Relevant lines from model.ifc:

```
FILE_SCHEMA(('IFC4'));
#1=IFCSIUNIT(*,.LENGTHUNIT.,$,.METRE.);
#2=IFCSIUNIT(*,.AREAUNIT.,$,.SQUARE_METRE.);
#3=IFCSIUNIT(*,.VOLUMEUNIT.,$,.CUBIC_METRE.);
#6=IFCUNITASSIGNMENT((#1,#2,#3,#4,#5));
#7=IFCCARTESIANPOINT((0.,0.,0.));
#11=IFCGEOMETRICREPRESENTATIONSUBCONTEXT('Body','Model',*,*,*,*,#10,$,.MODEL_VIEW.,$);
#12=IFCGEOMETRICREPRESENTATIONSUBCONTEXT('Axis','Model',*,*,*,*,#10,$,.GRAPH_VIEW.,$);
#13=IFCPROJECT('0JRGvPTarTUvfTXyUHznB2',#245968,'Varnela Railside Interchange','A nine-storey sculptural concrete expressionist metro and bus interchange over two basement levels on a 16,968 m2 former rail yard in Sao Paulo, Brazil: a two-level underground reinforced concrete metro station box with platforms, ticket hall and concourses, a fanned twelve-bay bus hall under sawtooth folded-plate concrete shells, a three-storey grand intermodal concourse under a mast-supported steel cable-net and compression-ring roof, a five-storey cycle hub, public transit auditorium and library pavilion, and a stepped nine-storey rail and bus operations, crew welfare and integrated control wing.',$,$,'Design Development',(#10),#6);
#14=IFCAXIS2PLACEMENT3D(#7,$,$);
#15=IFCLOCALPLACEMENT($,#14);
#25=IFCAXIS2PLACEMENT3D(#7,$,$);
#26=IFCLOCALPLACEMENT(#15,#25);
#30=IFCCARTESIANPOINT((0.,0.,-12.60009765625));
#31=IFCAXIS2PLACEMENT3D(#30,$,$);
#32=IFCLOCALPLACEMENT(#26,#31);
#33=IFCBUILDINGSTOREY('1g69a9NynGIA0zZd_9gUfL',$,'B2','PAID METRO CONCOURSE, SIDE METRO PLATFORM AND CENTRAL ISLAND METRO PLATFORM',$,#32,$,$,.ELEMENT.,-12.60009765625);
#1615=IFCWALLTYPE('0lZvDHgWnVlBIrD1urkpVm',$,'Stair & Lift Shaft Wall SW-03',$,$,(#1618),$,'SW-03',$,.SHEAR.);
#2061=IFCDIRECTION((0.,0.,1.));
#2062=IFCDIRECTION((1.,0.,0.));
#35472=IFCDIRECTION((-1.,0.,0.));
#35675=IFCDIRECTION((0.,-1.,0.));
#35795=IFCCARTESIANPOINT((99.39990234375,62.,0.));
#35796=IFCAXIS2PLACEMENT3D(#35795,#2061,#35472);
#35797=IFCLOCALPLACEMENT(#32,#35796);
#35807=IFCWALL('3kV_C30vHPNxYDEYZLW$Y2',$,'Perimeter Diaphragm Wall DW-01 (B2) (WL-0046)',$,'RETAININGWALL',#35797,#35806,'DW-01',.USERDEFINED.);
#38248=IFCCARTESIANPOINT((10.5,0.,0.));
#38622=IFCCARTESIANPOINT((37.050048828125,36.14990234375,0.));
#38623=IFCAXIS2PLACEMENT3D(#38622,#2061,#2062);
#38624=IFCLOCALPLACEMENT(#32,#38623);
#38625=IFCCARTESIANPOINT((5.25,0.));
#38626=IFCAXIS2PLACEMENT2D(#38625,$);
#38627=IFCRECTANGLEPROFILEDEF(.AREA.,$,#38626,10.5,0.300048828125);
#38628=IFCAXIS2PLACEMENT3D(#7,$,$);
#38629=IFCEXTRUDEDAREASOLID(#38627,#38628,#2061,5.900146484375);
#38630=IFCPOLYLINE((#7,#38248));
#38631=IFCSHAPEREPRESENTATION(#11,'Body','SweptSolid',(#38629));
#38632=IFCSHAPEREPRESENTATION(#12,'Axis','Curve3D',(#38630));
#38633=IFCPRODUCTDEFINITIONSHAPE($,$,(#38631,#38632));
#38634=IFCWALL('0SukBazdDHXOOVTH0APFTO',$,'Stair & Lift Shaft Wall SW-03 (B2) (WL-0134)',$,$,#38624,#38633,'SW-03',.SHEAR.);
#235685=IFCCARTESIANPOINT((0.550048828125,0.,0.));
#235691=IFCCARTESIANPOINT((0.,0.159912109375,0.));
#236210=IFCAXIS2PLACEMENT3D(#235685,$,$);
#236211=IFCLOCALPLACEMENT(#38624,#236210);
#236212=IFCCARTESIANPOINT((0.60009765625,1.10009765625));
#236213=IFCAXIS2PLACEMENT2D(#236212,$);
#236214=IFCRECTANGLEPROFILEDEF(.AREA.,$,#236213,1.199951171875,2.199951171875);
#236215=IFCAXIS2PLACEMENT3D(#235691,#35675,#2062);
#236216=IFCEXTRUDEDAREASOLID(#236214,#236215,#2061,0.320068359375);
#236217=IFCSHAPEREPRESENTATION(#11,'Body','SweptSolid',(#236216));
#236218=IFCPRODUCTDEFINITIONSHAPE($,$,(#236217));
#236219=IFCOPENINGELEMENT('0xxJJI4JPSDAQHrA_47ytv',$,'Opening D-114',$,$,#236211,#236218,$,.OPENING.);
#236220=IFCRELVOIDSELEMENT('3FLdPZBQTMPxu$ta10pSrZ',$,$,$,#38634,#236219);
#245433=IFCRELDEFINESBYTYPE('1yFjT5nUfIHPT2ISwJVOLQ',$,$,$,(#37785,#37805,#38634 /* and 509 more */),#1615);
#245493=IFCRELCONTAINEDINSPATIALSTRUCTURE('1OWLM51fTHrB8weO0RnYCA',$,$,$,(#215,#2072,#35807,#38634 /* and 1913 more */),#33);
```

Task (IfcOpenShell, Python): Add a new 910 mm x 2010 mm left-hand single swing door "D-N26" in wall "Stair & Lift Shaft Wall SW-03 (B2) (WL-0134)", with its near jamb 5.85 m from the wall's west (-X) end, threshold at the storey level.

```python
import numpy as np
import ifcopenshell
import ifcopenshell.api.feature
import ifcopenshell.api.geometry
import ifcopenshell.api.root
import ifcopenshell.api.spatial
import ifcopenshell.geom
import ifcopenshell.util.element
import ifcopenshell.util.placement
import ifcopenshell.util.representation
import ifcopenshell.util.shape
import ifcopenshell.util.unit

model = ifcopenshell.open("model.ifc")
unit_scale = ifcopenshell.util.unit.calculate_unit_scale(model)
settings = ifcopenshell.geom.settings()


def volume(element):
    """Net volume in cubic metres, openings subtracted."""
    shape = ifcopenshell.geom.create_shape(settings, element)
    return ifcopenshell.util.shape.get_volume(shape.geometry)


wall = model.by_guid("0SukBazdDHXOOVTH0APFTO")
storey = ifcopenshell.util.element.get_container(wall, ifc_class="IfcBuildingStorey")
context = ifcopenshell.util.representation.get_context(model, "Model", "Body", "MODEL_VIEW")
before = volume(wall)

width, height, from_end, sill = 0.91, 2.01, 5.85, 0.0  # metres

# The wall runs along its own X axis, and the end named is its -X end.
wall_shape = ifcopenshell.geom.create_shape(settings, wall)
x, y, z = ifcopenshell.util.shape.get_vertices(wall_shape.geometry).T
start = x.min() + from_end
face, thickness = float(y.min()), float(y.max() - y.min())
wall_matrix = ifcopenshell.util.placement.get_local_placement(wall.ObjectPlacement)
level = ifcopenshell.util.placement.get_local_placement(storey.ObjectPlacement)[2, 3]


def in_wall(x, y):
    """Placement at x, y metres in the wall's axes, at sill height."""
    matrix = wall_matrix.copy()
    matrix[:, 3] = wall_matrix @ np.array([x / unit_scale, y / unit_scale, 0.0, 1.0])
    matrix[2, 3] = level + sill / unit_scale
    return matrix


# Opening: a box that overshoots both wall faces by 50 mm.
opening = ifcopenshell.api.root.create_entity(model, ifc_class="IfcOpeningElement", predefined_type="OPENING")
box = ifcopenshell.api.geometry.add_wall_representation(
    model, context=context, length=width, height=height, thickness=thickness + 0.1
)
ifcopenshell.api.geometry.assign_representation(model, product=opening, representation=box)
ifcopenshell.api.geometry.edit_object_placement(model, product=opening, matrix=in_wall(start, face - 0.05), is_si=False)
ifcopenshell.api.feature.add_feature(model, feature=opening, element=wall)

door = ifcopenshell.api.root.create_entity(model, ifc_class="IfcDoor", name="D-N26", predefined_type="DOOR")
door.OverallWidth, door.OverallHeight = width / unit_scale, height / unit_scale
door.OperationType = "SINGLE_SWING_LEFT"
body = ifcopenshell.api.geometry.add_door_representation(
    model,
    context=context,
    overall_width=door.OverallWidth,
    overall_height=door.OverallHeight,
    operation_type="SINGLE_SWING_LEFT",
    lining_properties={"LiningDepth": thickness / unit_scale, "ThresholdDepth": thickness / unit_scale},
)
ifcopenshell.api.geometry.assign_representation(model, product=door, representation=body)
ifcopenshell.api.spatial.assign_container(model, products=[door], relating_structure=storey)
ifcopenshell.api.feature.add_filling(model, opening=opening, element=door)

# The lining spans the wall, so the door starts at the wall face.
ifcopenshell.api.geometry.edit_object_placement(model, product=door, matrix=in_wall(start, face), is_si=False)

after = volume(wall)

print(f"wall volume {before:.3f} -> {after:.3f} m3")

model.write("model_v2.ifc")
```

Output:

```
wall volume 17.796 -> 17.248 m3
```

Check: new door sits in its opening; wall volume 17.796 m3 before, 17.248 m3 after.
